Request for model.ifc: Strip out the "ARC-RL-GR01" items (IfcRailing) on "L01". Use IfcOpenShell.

First a look at what the model holds.

```python
import ifcopenshell
import ifcopenshell.util.element

model = ifcopenshell.open("model.ifc")
print(model.schema)
storey = next(s for s in model.by_type("IfcBuildingStorey") if s.Name == "L01")
railings = [e for e in ifcopenshell.util.element.get_decomposition(storey) if e.is_a("IfcRailing")]
seen = {}
for e in railings:
    element_type = ifcopenshell.util.element.get_type(e)
    name = element_type.Name if element_type not in (None, e) else None
    seen[name] = seen.get(name, 0) + 1
for name, count in sorted(seen.items(), key=str):
    print(count, "x", name)
```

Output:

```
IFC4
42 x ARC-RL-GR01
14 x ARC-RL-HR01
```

```python
import ifcopenshell
import ifcopenshell.api.root
import ifcopenshell.util.element

model = ifcopenshell.open("model.ifc")

storey = next(s for s in model.by_type("IfcBuildingStorey") if s.Name == "L01")
railings = [e for e in ifcopenshell.util.element.get_decomposition(storey) if e.is_a("IfcRailing")]
targets = [e for e in railings if (t := ifcopenshell.util.element.get_type(e)) not in (None, e) and t.Name == "ARC-RL-GR01"]

for e in targets:
    ifcopenshell.api.root.remove_product(model, product=e)
print(len(targets), "removed")

model.write("model_rev.ifc")
```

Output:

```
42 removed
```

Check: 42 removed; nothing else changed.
